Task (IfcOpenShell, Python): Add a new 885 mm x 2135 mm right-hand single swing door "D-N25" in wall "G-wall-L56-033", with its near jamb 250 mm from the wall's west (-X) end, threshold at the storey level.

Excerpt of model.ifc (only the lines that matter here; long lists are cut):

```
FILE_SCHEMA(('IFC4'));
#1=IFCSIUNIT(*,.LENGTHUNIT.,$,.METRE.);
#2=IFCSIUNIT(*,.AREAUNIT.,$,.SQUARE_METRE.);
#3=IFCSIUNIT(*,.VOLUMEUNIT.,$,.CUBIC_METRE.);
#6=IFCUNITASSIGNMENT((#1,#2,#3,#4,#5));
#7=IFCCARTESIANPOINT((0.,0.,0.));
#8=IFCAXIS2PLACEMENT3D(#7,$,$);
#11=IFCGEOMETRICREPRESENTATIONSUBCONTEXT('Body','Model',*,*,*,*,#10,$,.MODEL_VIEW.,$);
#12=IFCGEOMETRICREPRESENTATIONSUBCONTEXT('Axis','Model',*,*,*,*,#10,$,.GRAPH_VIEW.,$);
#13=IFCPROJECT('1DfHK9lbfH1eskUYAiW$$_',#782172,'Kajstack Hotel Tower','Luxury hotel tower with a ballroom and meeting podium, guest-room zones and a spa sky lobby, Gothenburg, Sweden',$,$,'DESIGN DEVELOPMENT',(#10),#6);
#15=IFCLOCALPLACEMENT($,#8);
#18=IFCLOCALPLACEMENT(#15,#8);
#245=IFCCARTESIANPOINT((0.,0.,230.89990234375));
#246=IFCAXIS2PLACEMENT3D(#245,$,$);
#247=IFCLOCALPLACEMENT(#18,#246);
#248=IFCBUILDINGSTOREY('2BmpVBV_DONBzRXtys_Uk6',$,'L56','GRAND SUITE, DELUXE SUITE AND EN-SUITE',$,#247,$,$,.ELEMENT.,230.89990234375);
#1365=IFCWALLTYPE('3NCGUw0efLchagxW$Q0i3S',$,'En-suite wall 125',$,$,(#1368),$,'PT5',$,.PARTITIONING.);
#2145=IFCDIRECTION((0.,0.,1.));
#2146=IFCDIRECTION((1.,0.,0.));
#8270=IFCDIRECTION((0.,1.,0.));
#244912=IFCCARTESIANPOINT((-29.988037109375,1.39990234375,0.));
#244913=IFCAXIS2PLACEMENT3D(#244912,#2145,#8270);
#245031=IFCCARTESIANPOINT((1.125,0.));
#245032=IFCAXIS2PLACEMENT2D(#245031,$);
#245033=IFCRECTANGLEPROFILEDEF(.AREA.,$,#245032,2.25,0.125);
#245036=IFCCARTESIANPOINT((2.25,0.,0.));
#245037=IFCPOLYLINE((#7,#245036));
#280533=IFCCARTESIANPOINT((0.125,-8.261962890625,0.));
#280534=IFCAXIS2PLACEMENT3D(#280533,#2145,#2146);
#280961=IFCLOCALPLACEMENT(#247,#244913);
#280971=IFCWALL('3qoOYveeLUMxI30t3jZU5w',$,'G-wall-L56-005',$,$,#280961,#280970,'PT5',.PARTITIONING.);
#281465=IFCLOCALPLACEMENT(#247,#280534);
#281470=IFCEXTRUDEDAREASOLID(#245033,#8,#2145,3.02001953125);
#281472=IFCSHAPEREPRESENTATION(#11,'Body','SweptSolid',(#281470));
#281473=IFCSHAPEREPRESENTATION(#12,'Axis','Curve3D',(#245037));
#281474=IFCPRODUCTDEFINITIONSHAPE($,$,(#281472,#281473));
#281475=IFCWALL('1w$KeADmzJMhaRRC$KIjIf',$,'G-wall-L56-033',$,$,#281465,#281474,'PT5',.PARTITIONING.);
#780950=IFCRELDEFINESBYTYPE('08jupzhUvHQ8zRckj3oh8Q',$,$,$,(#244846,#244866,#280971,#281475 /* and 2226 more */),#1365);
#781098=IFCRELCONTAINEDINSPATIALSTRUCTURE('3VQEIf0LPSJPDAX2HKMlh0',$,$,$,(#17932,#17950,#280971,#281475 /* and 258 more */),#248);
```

```python
import numpy as np
import ifcopenshell
import ifcopenshell.api.feature
import ifcopenshell.api.geometry
import ifcopenshell.api.root
import ifcopenshell.api.spatial
import ifcopenshell.geom
import ifcopenshell.util.element
import ifcopenshell.util.placement
import ifcopenshell.util.representation
import ifcopenshell.util.shape
import ifcopenshell.util.unit

model = ifcopenshell.open("model.ifc")
unit_scale = ifcopenshell.util.unit.calculate_unit_scale(model)
settings = ifcopenshell.geom.settings()


def volume(element):
    """Net volume in cubic metres, openings subtracted."""
    shape = ifcopenshell.geom.create_shape(settings, element)
    return ifcopenshell.util.shape.get_volume(shape.geometry)


wall = model.by_guid("1w$KeADmzJMhaRRC$KIjIf")
storey = ifcopenshell.util.element.get_container(wall, ifc_class="IfcBuildingStorey")
context = ifcopenshell.util.representation.get_context(model, "Model", "Body", "MODEL_VIEW")
before = volume(wall)

width, height, from_end, sill = 0.885, 2.135, 0.25, 0.0  # metres

# The wall runs along its own X axis, and the end named is its -X end.
wall_shape = ifcopenshell.geom.create_shape(settings, wall)
x, y, z = ifcopenshell.util.shape.get_vertices(wall_shape.geometry).T
start = x.min() + from_end
face, thickness = float(y.min()), float(y.max() - y.min())
wall_matrix = ifcopenshell.util.placement.get_local_placement(wall.ObjectPlacement)
level = ifcopenshell.util.placement.get_local_placement(storey.ObjectPlacement)[2, 3]


def in_wall(x, y):
    """Placement at x, y metres in the wall's axes, at sill height."""
    matrix = wall_matrix.copy()
    matrix[:, 3] = wall_matrix @ np.array([x / unit_scale, y / unit_scale, 0.0, 1.0])
    matrix[2, 3] = level + sill / unit_scale
    return matrix


# Opening: a box that overshoots both wall faces by 50 mm.
opening = ifcopenshell.api.root.create_entity(model, ifc_class="IfcOpeningElement", predefined_type="OPENING")
box = ifcopenshell.api.geometry.add_wall_representation(
    model, context=context, length=width, height=height, thickness=thickness + 0.1
)
ifcopenshell.api.geometry.assign_representation(model, product=opening, representation=box)
ifcopenshell.api.geometry.edit_object_placement(model, product=opening, matrix=in_wall(start, face - 0.05), is_si=False)
ifcopenshell.api.feature.add_feature(model, feature=opening, element=wall)

door = ifcopenshell.api.root.create_entity(model, ifc_class="IfcDoor", name="D-N25", predefined_type="DOOR")
door.OverallWidth, door.OverallHeight = width / unit_scale, height / unit_scale
door.OperationType = "SINGLE_SWING_RIGHT"
body = ifcopenshell.api.geometry.add_door_representation(
    model,
    context=context,
    overall_width=door.OverallWidth,
    overall_height=door.OverallHeight,
    operation_type="SINGLE_SWING_RIGHT",
    lining_properties={"LiningDepth": thickness / unit_scale, "ThresholdDepth": thickness / unit_scale},
)
ifcopenshell.api.geometry.assign_representation(model, product=door, representation=body)
ifcopenshell.api.spatial.assign_container(model, products=[door], relating_structure=storey)
ifcopenshell.api.feature.add_filling(model, opening=opening, element=door)

# The lining spans the wall, so the door starts at the wall face.
ifcopenshell.api.geometry.edit_object_placement(model, product=door, matrix=in_wall(start, face), is_si=False)

after = volume(wall)

print(f"wall volume {before:.3f} -> {after:.3f} m3")

model.write("model_rev.ifc")
```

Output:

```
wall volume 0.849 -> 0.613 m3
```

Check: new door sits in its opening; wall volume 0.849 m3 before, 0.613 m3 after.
